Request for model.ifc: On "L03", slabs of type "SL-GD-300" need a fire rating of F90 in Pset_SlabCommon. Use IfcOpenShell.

First a look at what the model holds.

```python
import ifcopenshell
import ifcopenshell.util.element

model = ifcopenshell.open("model.ifc")
print(model.schema)
storey = next(s for s in model.by_type("IfcBuildingStorey") if s.Name == "L03")
slabs = [e for e in ifcopenshell.util.element.get_decomposition(storey) if e.is_a("IfcSlab")]
seen = {}
for e in slabs:
    element_type = ifcopenshell.util.element.get_type(e)
    key = (element_type.Name if element_type != e and element_type else None, ifcopenshell.util.element.get_pset(e, "Pset_SlabCommon", "FireRating"))
    seen[key] = seen.get(key, 0) + 1
for (name, value), count in sorted(seen.items(), key=str):
    print(count, "x", name, "|", value)
```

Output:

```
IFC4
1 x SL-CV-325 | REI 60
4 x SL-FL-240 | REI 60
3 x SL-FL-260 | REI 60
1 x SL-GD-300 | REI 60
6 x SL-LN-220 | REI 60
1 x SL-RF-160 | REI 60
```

```python
import ifcopenshell
import ifcopenshell.api.pset
import ifcopenshell.util.element

model = ifcopenshell.open("model.ifc")

storey = next(s for s in model.by_type("IfcBuildingStorey") if s.Name == "L03")
slabs = [e for e in ifcopenshell.util.element.get_decomposition(storey) if e.is_a("IfcSlab")]

count = 0
for e in slabs:
    element_type = ifcopenshell.util.element.get_type(e)
    if element_type in (None, e) or element_type.Name != "SL-GD-300":
        continue
    # add_pset returns the element's existing set when there is one.
    pset = ifcopenshell.api.pset.add_pset(model, product=e, name="Pset_SlabCommon")
    ifcopenshell.api.pset.edit_pset(model, pset=pset, properties={"FireRating": "F90"})
    count += 1

print(count, "slabs updated")

model.write("model_rev.ifc")
```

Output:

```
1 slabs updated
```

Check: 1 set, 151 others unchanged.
